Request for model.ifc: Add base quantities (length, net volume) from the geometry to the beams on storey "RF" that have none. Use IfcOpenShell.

First a look at what the model holds.

```python
import ifcopenshell
import ifcopenshell.util.element
import ifcopenshell.util.unit

model = ifcopenshell.open("model.ifc")
print(model.schema)
for unit_type in ("LENGTHUNIT", "AREAUNIT", "VOLUMEUNIT"):
    print(unit_type, ifcopenshell.util.unit.calculate_unit_scale(model, unit_type))
storey = next(s for s in model.by_type("IfcBuildingStorey") if s.Name == "RF")
beams = [e for e in ifcopenshell.util.element.get_decomposition(storey) if e.is_a("IfcBeam")]
for e in sorted(beams, key=lambda e: e.id()):
    print(e.id(), e.is_a(), e.Name, list(ifcopenshell.util.element.get_psets(e, qtos_only=True)), sep=" | ")
```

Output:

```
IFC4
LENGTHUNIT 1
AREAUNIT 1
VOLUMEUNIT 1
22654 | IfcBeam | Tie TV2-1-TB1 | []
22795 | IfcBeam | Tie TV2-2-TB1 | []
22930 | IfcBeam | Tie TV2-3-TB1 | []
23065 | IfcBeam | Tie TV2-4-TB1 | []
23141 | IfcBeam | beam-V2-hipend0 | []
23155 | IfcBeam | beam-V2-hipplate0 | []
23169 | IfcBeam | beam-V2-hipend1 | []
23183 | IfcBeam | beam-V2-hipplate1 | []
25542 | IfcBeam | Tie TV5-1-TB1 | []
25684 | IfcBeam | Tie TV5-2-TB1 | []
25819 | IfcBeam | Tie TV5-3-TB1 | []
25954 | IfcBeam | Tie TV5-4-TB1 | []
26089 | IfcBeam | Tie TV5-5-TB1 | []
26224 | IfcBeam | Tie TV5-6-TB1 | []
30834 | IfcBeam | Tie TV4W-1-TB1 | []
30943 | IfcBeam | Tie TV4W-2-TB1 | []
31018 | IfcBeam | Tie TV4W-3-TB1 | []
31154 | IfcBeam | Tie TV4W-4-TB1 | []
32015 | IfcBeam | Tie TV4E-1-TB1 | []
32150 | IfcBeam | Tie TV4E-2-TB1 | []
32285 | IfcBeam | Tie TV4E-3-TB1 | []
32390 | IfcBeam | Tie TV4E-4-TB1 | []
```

```python
import ifcopenshell
import ifcopenshell.api.pset
import ifcopenshell.geom
import ifcopenshell.util.element
import ifcopenshell.util.shape
import ifcopenshell.util.unit

model = ifcopenshell.open("model.ifc")
unit_scale = ifcopenshell.util.unit.calculate_unit_scale(model)
volume_scale = ifcopenshell.util.unit.calculate_unit_scale(model, "VOLUMEUNIT")
settings = ifcopenshell.geom.settings()

storey = next(s for s in model.by_type("IfcBuildingStorey") if s.Name == "RF")
beams = [e for e in ifcopenshell.util.element.get_decomposition(storey) if e.is_a("IfcBeam")]

for e in sorted(beams, key=lambda e: e.id()):
    if ifcopenshell.util.element.get_psets(e, qtos_only=True, should_inherit=False):
        continue
    # Geometry comes back in metres, in the element's own axes.
    shape = ifcopenshell.geom.create_shape(settings, e)
    values = {
        "Length": ifcopenshell.util.shape.get_max_xyz(shape.geometry) / unit_scale,
        "NetVolume": ifcopenshell.util.shape.get_volume(shape.geometry) / volume_scale,
    }
    qto = ifcopenshell.api.pset.add_qto(model, product=e, name="Qto_BeamBaseQuantities")
    ifcopenshell.api.pset.edit_qto(model, qto=qto, properties=values)
    print(e.id(), {k: round(v, 3) for k, v in values.items()})

model.write("model_v2.ifc")
```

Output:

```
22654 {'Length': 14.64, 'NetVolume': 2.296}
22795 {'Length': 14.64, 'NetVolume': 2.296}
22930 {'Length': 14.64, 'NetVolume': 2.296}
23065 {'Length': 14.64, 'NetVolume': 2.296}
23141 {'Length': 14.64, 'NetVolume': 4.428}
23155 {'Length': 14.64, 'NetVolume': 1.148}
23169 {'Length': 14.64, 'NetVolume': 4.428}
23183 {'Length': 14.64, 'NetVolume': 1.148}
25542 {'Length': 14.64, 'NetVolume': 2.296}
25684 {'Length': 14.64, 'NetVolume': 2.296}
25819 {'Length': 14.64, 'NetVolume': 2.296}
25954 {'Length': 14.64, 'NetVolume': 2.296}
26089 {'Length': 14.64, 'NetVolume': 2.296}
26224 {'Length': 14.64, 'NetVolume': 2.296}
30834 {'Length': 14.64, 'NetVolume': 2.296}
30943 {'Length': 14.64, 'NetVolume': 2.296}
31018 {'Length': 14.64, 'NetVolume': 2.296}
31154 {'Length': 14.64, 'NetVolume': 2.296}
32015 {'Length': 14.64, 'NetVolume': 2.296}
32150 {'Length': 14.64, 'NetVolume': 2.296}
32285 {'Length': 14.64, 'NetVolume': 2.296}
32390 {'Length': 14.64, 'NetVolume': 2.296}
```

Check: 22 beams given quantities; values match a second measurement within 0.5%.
